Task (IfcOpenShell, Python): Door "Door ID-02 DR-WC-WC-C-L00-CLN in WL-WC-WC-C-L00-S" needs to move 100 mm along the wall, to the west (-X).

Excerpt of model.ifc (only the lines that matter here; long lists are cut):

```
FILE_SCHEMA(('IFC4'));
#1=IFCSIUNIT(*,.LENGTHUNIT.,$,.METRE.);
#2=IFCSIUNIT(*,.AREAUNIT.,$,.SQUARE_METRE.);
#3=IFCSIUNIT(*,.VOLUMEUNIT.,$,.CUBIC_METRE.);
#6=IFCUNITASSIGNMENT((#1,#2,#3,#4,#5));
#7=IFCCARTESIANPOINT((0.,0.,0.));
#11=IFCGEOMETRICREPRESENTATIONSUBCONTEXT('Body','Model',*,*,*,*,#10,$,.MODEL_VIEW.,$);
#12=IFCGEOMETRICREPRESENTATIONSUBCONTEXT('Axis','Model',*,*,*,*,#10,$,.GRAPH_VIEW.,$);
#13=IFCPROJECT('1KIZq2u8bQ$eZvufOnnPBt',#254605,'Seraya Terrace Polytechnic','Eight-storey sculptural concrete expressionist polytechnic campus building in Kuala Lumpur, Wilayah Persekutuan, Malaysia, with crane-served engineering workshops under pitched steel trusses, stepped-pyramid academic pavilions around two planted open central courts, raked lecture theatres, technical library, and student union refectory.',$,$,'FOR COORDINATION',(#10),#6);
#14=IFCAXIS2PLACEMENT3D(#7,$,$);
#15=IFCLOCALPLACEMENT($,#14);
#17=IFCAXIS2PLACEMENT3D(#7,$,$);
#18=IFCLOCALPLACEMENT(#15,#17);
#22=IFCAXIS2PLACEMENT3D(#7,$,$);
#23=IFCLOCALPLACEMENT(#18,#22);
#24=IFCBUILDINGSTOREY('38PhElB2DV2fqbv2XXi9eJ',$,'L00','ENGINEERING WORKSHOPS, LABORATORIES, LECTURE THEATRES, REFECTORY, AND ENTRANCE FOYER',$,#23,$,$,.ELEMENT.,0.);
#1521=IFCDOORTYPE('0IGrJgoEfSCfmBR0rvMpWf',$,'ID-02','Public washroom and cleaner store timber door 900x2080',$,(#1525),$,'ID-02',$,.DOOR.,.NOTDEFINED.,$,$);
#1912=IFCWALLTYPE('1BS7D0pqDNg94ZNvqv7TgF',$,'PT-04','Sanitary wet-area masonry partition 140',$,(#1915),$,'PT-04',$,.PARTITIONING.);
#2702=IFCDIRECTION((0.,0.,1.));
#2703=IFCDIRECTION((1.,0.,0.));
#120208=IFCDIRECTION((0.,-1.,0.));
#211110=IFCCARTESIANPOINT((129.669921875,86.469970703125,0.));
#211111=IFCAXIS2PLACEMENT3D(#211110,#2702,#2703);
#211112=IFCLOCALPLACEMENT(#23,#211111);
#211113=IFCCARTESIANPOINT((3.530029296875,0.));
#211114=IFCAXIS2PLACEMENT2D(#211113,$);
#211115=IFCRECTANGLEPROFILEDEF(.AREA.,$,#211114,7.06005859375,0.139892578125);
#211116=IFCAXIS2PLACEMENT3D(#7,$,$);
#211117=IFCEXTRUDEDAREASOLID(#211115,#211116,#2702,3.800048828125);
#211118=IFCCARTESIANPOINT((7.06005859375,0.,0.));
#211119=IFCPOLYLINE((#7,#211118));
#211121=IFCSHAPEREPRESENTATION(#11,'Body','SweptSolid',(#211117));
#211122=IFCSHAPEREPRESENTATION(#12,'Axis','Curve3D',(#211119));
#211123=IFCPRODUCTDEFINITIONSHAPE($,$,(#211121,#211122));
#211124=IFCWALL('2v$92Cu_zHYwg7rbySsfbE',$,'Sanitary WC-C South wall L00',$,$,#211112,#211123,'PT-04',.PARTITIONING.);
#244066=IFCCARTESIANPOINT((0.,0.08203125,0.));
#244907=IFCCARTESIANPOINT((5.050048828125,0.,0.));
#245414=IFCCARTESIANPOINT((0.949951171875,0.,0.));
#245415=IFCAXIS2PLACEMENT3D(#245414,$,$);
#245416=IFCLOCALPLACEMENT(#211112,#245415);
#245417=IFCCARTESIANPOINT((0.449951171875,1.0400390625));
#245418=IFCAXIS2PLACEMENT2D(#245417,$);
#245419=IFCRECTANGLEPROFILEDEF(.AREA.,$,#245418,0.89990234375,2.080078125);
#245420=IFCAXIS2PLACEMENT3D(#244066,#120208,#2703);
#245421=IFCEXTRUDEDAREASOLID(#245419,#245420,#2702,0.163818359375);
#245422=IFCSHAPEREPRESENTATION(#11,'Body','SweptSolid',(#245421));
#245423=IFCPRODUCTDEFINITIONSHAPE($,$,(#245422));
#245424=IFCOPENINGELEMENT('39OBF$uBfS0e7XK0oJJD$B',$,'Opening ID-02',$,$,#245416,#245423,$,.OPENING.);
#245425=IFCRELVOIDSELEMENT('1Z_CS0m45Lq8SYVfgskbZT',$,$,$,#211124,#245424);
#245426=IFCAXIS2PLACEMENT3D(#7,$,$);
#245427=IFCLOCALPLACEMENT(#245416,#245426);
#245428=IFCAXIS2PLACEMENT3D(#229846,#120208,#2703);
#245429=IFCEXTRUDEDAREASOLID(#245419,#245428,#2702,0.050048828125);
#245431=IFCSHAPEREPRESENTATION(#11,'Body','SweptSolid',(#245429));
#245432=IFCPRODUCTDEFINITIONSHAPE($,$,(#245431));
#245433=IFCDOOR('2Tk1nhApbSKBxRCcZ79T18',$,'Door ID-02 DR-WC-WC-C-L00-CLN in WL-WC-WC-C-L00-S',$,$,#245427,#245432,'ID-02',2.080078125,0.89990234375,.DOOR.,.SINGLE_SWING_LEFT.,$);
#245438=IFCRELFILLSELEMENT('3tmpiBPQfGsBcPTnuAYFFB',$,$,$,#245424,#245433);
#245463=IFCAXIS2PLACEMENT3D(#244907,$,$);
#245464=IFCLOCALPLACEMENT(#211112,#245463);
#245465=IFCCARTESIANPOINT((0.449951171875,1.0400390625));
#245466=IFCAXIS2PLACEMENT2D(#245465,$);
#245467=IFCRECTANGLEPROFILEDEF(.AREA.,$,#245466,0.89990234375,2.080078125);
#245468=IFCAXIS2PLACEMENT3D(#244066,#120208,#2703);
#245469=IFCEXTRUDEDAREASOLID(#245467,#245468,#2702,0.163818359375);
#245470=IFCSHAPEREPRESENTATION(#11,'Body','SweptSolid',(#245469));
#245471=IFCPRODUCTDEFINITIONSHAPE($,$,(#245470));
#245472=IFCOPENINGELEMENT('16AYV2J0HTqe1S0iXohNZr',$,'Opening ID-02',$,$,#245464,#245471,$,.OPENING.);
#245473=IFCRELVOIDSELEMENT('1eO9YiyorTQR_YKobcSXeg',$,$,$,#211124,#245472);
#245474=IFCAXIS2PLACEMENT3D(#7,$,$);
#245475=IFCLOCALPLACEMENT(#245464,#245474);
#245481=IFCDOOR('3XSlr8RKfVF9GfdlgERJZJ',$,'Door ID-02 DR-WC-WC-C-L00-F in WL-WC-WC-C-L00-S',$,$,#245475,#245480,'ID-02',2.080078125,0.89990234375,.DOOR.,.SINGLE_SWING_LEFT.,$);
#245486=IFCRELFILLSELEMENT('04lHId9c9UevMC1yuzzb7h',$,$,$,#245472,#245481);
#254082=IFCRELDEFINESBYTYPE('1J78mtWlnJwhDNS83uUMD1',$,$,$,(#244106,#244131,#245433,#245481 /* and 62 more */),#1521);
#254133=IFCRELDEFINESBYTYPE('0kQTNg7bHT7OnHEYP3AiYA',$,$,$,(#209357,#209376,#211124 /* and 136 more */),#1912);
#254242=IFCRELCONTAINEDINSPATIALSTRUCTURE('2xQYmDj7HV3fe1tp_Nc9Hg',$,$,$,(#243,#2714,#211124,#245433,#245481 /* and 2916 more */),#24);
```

```python
import ifcopenshell
import ifcopenshell.api.geometry
import ifcopenshell.util.placement
import ifcopenshell.util.unit

model = ifcopenshell.open("model.ifc")
unit_scale = ifcopenshell.util.unit.calculate_unit_scale(model)

door = model.by_guid("2Tk1nhApbSKBxRCcZ79T18")
opening = door.FillsVoids[0].RelatingOpeningElement
wall = opening.VoidsElements[0].RelatingBuildingElement

wall_matrix = ifcopenshell.util.placement.get_local_placement(wall.ObjectPlacement)
shift = wall_matrix[:3, 0] * -0.1 / unit_scale
before = ifcopenshell.util.placement.get_local_placement(door.ObjectPlacement)[:3, 3].copy()

# The door is placed relative to its opening, so it follows when the opening moves.
matrix = ifcopenshell.util.placement.get_local_placement(opening.ObjectPlacement)
matrix[:3, 3] += shift
ifcopenshell.api.geometry.edit_object_placement(
    model, product=opening, matrix=matrix, is_si=False, should_transform_children=True
)

after = ifcopenshell.util.placement.get_local_placement(door.ObjectPlacement)[:3, 3]
print("door moved by", (after - before).round(3) + 0.0)

model.write("model_rev.ifc")
```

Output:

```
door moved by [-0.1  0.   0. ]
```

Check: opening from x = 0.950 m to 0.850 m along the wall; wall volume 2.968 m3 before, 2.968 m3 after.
